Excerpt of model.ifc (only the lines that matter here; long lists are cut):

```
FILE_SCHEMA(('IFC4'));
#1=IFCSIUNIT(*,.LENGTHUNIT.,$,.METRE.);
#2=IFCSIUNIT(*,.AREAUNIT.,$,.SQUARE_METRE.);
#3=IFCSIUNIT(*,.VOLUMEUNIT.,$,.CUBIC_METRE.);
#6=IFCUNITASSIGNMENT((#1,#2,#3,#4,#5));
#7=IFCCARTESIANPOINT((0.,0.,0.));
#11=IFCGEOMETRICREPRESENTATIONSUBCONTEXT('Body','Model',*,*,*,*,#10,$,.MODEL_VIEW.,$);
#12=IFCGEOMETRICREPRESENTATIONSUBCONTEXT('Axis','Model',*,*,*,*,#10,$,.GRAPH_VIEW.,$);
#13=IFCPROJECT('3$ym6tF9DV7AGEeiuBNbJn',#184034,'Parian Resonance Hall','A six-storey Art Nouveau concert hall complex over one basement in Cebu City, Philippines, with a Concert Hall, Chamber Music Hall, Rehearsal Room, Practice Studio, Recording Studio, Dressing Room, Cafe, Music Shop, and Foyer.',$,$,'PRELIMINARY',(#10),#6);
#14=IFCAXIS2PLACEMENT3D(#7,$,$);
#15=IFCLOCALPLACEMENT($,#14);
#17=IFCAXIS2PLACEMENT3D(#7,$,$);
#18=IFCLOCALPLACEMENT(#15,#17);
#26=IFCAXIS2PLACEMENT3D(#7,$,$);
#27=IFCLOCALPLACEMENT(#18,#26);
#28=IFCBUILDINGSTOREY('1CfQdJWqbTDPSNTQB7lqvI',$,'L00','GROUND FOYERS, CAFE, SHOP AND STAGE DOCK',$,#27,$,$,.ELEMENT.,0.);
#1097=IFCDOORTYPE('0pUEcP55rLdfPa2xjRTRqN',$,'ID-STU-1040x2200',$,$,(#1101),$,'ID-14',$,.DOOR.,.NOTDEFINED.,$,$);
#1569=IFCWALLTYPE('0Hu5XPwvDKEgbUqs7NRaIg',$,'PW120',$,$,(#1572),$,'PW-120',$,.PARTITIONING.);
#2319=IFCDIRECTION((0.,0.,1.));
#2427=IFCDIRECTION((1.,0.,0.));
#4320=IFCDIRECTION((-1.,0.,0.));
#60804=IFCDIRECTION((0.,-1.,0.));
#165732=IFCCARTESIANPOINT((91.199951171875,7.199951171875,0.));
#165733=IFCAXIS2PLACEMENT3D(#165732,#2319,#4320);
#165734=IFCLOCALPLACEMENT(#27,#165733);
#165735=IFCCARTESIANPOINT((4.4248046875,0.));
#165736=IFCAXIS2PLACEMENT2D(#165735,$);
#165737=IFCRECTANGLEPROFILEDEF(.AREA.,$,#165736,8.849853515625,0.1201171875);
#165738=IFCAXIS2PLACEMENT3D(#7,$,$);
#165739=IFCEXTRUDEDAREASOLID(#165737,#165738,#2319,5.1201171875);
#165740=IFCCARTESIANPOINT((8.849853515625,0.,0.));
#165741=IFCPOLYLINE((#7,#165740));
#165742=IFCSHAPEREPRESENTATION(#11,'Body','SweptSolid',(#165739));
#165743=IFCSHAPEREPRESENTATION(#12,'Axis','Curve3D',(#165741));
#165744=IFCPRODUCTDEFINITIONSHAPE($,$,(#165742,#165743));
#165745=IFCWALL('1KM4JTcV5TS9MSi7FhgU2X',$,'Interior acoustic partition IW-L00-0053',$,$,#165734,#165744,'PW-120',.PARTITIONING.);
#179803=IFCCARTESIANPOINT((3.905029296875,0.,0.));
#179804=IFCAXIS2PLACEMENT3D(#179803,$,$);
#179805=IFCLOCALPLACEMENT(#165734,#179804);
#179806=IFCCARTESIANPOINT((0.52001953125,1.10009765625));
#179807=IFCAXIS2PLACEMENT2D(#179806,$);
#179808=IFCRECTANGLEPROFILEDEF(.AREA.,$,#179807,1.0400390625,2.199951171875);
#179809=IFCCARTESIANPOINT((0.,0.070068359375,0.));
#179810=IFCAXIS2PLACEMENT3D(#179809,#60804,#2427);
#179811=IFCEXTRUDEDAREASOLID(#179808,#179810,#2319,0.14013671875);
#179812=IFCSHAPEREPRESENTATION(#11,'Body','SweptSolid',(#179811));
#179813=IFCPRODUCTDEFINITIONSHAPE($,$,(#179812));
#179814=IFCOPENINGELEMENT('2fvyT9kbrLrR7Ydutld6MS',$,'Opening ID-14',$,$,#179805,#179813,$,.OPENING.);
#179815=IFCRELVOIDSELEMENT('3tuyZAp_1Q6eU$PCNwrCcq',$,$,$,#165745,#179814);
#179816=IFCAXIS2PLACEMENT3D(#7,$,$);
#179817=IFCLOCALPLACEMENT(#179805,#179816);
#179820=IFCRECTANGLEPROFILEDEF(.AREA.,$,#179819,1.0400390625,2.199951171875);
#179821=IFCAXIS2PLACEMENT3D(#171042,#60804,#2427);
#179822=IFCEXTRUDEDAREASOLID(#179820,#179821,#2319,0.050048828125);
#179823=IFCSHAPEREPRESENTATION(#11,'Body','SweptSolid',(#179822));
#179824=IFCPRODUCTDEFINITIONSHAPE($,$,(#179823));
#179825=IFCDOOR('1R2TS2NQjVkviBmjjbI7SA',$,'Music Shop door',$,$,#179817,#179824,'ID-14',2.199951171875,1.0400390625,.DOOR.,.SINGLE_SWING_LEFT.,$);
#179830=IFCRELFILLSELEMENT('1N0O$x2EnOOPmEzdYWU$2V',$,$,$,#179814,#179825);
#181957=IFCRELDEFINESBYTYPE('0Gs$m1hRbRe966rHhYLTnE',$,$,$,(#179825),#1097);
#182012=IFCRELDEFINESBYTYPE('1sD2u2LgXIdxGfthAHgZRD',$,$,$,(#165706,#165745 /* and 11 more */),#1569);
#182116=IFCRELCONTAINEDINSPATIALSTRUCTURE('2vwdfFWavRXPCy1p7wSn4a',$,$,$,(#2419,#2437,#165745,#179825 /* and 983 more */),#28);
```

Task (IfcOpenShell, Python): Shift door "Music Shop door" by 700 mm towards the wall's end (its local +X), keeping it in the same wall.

```python
import ifcopenshell
import ifcopenshell.api.geometry
import ifcopenshell.util.placement
import ifcopenshell.util.unit

model = ifcopenshell.open("model.ifc")
unit_scale = ifcopenshell.util.unit.calculate_unit_scale(model)

door = model.by_guid("1R2TS2NQjVkviBmjjbI7SA")
opening = door.FillsVoids[0].RelatingOpeningElement
wall = opening.VoidsElements[0].RelatingBuildingElement

wall_matrix = ifcopenshell.util.placement.get_local_placement(wall.ObjectPlacement)
shift = wall_matrix[:3, 0] * 0.7 / unit_scale
before = ifcopenshell.util.placement.get_local_placement(door.ObjectPlacement)[:3, 3].copy()

# The door is placed relative to its opening, so it follows when the opening moves.
matrix = ifcopenshell.util.placement.get_local_placement(opening.ObjectPlacement)
matrix[:3, 3] += shift
ifcopenshell.api.geometry.edit_object_placement(
    model, product=opening, matrix=matrix, is_si=False, should_transform_children=True
)

after = ifcopenshell.util.placement.get_local_placement(door.ObjectPlacement)[:3, 3]
print("door moved by", (after - before).round(3) + 0.0)

model.write("model_v2.ifc")
```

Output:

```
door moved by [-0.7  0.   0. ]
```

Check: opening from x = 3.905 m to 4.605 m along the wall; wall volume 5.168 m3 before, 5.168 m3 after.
